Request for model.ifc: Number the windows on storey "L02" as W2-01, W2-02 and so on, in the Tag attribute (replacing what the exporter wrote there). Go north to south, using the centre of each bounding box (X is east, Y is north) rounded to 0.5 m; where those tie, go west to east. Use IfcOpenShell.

First a look at what the model holds.

```python
import ifcopenshell
import ifcopenshell.util.element
import ifcopenshell.util.placement

model = ifcopenshell.open("model.ifc")
print(model.schema)
storey = next(s for s in model.by_type("IfcBuildingStorey") if s.Name == "L02")
windows = [e for e in ifcopenshell.util.element.get_decomposition(storey) if e.is_a("IfcWindow")]
for e in sorted(windows, key=lambda e: e.id()):
    origin = ifcopenshell.util.placement.get_local_placement(e.ObjectPlacement)[:3, 3]
    print(e.id(), e.Tag, e.Name, origin.round(2) + 0.0, sep=" | ")
```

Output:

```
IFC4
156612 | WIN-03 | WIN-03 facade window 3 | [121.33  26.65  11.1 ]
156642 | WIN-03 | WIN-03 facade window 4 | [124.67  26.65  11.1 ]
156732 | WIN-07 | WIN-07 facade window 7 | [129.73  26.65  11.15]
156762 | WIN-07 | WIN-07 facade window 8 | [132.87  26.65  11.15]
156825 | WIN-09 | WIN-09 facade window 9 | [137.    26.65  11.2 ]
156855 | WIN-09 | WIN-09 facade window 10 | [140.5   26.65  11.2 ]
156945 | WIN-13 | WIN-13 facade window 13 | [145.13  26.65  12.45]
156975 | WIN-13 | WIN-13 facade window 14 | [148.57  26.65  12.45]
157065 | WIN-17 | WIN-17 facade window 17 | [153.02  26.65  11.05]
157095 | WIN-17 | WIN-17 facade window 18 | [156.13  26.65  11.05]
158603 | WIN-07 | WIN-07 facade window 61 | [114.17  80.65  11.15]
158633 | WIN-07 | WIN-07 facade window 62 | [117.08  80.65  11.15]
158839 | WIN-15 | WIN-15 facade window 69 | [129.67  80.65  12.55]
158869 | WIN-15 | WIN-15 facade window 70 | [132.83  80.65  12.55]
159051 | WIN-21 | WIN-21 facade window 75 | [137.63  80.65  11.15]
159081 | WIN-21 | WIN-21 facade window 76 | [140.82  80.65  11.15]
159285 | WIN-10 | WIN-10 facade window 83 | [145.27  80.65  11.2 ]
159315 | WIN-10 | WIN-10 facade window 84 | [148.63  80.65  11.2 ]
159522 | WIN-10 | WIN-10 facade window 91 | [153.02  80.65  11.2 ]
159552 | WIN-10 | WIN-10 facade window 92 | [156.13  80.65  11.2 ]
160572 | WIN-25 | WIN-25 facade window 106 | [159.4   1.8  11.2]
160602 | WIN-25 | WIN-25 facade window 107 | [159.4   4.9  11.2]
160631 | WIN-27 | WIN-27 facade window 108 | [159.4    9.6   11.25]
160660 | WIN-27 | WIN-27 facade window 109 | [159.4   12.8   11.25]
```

```python
import ifcopenshell
import ifcopenshell.geom
import ifcopenshell.util.element
import ifcopenshell.util.shape

model = ifcopenshell.open("model.ifc")
settings = ifcopenshell.geom.settings()
settings.set("use-world-coords", True)


def centre(element):
    shape = ifcopenshell.geom.create_shape(settings, element)
    return ifcopenshell.util.shape.get_bbox_centroid(shape.geometry)


storey = next(s for s in model.by_type("IfcBuildingStorey") if s.Name == "L02")
windows = [e for e in ifcopenshell.util.element.get_decomposition(storey) if e.is_a("IfcWindow")]

# Insertion points can sit at a corner or the storey origin, so sort by the geometry (in metres).
centres = {e: centre(e) for e in windows}
windows.sort(key=lambda e: (-round(centres[e][1] / 0.5), centres[e][0]))

for i, e in enumerate(windows, start=1):
    number = f"W2-{i:02d}"
    e.Tag = number
    print(e.id(), number)

model.write("model_updated.ifc")
```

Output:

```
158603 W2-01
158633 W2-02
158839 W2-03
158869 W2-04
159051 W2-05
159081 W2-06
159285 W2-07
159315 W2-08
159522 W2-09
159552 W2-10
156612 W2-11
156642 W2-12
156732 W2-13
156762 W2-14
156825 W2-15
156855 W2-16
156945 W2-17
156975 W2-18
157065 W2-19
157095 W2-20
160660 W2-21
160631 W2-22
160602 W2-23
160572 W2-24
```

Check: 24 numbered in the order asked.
